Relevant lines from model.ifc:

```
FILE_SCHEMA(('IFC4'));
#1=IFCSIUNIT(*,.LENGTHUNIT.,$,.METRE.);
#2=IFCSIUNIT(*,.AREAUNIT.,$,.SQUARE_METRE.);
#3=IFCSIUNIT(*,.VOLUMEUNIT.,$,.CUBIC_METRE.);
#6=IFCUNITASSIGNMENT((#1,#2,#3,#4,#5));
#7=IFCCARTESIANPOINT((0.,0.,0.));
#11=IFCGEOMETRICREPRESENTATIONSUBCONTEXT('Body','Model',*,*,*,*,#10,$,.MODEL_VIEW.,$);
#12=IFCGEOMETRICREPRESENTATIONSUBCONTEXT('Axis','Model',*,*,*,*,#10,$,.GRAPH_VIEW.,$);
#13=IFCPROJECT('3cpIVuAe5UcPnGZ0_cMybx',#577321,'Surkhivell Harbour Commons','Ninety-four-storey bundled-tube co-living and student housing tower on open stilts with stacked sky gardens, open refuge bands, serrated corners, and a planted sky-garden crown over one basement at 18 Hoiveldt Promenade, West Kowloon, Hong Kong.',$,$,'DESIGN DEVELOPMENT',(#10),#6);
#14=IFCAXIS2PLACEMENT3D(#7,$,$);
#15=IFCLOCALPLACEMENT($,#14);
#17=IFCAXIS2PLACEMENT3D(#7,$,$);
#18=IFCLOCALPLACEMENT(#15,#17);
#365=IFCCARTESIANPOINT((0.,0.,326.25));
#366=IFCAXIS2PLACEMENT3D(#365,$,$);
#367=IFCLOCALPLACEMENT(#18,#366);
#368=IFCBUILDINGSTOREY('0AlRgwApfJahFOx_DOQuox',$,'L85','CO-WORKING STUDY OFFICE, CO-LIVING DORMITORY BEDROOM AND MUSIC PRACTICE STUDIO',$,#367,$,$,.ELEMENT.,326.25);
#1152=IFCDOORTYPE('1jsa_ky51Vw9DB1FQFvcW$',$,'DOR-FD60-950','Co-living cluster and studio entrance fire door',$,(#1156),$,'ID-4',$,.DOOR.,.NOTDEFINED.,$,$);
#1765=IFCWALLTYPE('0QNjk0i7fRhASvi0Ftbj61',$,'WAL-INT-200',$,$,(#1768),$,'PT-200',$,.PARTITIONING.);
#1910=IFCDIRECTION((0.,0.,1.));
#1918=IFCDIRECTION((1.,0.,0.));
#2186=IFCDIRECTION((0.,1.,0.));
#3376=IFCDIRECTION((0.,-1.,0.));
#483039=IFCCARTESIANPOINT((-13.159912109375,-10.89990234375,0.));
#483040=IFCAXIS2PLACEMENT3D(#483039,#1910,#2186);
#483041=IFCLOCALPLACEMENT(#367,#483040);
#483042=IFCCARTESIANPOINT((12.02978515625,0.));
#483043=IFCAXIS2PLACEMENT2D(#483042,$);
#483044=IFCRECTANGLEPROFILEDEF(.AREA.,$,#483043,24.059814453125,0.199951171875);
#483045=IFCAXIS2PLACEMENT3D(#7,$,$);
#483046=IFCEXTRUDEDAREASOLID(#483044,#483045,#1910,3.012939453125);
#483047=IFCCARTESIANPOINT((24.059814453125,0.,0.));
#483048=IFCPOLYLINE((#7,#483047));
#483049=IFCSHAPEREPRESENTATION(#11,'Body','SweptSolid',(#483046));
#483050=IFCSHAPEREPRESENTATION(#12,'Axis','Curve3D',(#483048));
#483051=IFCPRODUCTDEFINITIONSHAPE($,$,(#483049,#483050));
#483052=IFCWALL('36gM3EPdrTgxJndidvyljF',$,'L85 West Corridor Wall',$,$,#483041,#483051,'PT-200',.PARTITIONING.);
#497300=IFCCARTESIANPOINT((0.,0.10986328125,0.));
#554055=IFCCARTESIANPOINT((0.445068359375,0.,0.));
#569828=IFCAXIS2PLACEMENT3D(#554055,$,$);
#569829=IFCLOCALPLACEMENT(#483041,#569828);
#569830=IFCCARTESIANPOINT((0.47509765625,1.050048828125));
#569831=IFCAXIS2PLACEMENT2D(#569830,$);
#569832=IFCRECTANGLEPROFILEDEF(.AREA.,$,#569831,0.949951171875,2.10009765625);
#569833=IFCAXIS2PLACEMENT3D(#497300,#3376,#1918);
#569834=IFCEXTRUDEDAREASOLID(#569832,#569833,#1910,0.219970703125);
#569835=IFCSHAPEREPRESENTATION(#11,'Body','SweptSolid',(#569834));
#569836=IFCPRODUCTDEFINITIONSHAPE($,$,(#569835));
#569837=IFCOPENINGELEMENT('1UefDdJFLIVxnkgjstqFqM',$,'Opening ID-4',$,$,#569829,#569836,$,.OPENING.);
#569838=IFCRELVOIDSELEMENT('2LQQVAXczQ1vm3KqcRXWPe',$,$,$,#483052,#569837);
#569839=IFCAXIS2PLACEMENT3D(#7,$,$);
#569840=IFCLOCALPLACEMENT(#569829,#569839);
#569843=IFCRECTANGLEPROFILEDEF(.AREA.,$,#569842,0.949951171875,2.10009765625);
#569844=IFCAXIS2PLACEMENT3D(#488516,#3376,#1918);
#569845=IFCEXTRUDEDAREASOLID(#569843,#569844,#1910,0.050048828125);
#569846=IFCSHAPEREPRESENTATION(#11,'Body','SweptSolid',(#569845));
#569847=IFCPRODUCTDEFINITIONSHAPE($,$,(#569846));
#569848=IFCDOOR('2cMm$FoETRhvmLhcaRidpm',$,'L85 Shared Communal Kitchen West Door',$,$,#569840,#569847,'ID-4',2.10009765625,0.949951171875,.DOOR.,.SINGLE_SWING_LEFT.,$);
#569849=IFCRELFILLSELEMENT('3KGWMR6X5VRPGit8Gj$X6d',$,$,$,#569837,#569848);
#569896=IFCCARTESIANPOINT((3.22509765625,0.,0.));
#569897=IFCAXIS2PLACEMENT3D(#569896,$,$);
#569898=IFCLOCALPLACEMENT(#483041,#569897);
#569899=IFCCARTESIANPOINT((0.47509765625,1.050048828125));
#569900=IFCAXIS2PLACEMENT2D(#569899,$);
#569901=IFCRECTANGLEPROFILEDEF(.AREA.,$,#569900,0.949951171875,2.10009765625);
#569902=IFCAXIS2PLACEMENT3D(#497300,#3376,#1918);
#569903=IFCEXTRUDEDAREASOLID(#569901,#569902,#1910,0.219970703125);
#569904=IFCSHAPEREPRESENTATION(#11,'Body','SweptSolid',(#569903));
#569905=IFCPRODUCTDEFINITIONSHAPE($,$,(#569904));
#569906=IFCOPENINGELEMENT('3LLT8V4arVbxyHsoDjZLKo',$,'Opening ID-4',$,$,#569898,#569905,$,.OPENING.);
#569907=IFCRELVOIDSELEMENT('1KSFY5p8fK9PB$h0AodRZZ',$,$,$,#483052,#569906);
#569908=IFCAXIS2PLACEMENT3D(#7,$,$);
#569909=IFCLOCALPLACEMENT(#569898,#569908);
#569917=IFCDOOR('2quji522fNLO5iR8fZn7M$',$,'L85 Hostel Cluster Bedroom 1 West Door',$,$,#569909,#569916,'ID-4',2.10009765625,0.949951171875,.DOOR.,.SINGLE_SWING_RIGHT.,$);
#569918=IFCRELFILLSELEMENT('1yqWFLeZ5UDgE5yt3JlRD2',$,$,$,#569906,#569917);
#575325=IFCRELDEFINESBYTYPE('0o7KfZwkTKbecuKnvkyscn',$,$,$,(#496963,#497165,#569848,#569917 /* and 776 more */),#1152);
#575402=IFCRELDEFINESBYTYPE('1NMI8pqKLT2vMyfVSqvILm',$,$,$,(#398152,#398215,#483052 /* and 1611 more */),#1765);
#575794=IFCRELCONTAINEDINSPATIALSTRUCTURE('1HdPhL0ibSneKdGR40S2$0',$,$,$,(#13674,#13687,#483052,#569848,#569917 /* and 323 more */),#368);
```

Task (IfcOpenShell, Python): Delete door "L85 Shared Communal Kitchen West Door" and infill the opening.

```python
import ifcopenshell
import ifcopenshell.api.feature
import ifcopenshell.api.root
import ifcopenshell.geom
import ifcopenshell.util.shape

model = ifcopenshell.open("model.ifc")
settings = ifcopenshell.geom.settings()


def volume(element):
    """Net volume in cubic metres, openings subtracted."""
    shape = ifcopenshell.geom.create_shape(settings, element)
    return ifcopenshell.util.shape.get_volume(shape.geometry)


door = model.by_guid("2cMm$FoETRhvmLhcaRidpm")
opening = door.FillsVoids[0].RelatingOpeningElement
wall = opening.VoidsElements[0].RelatingBuildingElement
before = volume(wall)

ifcopenshell.api.root.remove_product(model, product=door)
ifcopenshell.api.feature.remove_feature(model, feature=opening)

after = volume(wall)

print(f"wall volume {before:.3f} -> {after:.3f} m3")

model.write("model_rev.ifc")
```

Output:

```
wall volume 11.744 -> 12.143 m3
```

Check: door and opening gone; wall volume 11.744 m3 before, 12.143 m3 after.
